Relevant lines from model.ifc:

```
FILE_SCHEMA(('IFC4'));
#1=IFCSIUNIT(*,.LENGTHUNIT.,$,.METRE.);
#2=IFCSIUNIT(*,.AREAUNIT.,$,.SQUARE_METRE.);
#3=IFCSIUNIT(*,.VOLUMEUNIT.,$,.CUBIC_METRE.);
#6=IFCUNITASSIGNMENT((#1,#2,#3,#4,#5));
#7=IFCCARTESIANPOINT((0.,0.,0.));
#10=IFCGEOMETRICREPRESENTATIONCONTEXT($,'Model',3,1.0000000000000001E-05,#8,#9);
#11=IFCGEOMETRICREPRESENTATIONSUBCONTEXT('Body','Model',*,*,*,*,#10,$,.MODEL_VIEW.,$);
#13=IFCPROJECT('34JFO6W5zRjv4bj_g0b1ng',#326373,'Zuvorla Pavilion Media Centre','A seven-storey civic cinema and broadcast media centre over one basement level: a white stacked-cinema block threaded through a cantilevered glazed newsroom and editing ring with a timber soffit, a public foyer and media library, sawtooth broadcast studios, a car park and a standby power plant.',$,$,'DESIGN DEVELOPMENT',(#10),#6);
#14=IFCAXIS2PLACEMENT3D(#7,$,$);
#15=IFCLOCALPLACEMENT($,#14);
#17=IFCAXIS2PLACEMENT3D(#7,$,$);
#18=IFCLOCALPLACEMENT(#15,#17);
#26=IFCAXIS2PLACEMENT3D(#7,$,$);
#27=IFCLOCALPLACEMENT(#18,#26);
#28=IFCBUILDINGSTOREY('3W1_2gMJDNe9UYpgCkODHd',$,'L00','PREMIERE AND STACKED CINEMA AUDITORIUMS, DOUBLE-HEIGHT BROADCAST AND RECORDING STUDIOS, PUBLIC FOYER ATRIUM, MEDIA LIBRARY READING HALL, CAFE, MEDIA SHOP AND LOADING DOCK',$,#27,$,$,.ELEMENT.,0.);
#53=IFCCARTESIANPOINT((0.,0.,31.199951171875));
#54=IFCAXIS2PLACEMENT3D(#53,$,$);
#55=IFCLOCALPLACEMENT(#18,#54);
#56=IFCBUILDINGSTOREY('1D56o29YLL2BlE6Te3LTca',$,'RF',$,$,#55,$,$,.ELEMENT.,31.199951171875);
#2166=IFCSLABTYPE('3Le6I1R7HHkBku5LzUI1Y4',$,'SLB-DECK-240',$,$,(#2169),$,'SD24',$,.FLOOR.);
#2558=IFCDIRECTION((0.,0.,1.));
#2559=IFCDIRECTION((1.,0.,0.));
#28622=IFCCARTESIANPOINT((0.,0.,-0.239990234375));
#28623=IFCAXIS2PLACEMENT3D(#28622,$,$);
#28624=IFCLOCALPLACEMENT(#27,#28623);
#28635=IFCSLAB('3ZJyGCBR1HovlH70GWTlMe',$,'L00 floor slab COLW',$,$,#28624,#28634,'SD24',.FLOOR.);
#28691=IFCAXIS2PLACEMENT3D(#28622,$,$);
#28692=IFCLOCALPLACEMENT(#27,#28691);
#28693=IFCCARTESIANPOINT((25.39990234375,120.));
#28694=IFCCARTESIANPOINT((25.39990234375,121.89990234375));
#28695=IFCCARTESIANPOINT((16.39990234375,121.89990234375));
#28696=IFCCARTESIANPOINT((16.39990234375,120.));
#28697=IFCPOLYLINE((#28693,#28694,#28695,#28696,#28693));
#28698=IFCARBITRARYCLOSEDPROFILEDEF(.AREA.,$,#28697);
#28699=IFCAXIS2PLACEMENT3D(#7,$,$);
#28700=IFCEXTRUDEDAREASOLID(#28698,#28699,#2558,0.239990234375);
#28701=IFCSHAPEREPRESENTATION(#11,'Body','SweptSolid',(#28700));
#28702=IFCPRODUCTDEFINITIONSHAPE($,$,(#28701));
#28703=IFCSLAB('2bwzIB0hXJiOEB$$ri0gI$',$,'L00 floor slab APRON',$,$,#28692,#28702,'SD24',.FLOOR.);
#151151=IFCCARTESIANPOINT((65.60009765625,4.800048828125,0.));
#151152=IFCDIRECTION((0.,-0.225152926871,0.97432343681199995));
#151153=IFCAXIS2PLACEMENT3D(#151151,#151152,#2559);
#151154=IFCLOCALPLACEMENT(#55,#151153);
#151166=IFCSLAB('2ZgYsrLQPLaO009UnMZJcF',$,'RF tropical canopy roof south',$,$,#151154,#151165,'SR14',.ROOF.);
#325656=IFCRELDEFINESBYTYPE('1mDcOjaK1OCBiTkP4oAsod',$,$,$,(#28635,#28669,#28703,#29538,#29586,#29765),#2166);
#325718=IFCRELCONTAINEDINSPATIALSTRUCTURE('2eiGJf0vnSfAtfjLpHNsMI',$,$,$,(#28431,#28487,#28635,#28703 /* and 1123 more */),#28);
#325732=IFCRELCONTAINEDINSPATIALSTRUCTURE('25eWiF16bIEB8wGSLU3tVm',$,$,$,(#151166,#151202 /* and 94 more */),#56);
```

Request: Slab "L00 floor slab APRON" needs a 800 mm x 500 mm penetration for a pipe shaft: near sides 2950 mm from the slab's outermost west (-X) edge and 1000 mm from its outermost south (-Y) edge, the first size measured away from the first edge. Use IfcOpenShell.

```python
import numpy as np
import ifcopenshell
import ifcopenshell.api.feature
import ifcopenshell.api.geometry
import ifcopenshell.api.root
import ifcopenshell.geom
import ifcopenshell.util.placement
import ifcopenshell.util.representation
import ifcopenshell.util.shape
import ifcopenshell.util.unit

model = ifcopenshell.open("model.ifc")
unit_scale = ifcopenshell.util.unit.calculate_unit_scale(model)
settings = ifcopenshell.geom.settings()


def volume(element):
    """Net volume in cubic metres, openings subtracted."""
    shape = ifcopenshell.geom.create_shape(settings, element)
    return ifcopenshell.util.shape.get_volume(shape.geometry)


slab = model.by_guid("2bwzIB0hXJiOEB$$ri0gI$")
before = volume(slab)

# Extent in the slab's own axes, in metres. The edges named are its -X and -Y sides.
slab_shape = ifcopenshell.geom.create_shape(settings, slab)
vertices = ifcopenshell.util.shape.get_vertices(slab_shape.geometry)
x_min, y_min, bottom = vertices.min(axis=0)
top = vertices[:, 2].max()

opening = ifcopenshell.api.root.create_entity(model, ifc_class="IfcOpeningElement", name="Pipe shaft opening", predefined_type="OPENING")
context = ifcopenshell.util.representation.get_context(model, "Model", "Body", "MODEL_VIEW")
width, depth = 0.8, 0.5
outline = [(0.0, 0.0), (width, 0.0), (width, depth), (0.0, depth), (0.0, 0.0)]
# Overshoot both faces by 50 mm so the cut is clean.
shape = ifcopenshell.api.geometry.add_slab_representation(
    model, context=context, depth=top - bottom + 0.1, polyline=outline
)
ifcopenshell.api.geometry.assign_representation(model, product=opening, representation=shape)

matrix = ifcopenshell.util.placement.get_local_placement(slab.ObjectPlacement)
matrix[:, 3] = matrix @ np.append(np.array([x_min + 2.95, y_min + 1, bottom - 0.05]) / unit_scale, 1.0)
ifcopenshell.api.geometry.edit_object_placement(model, product=opening, matrix=matrix, is_si=False)
ifcopenshell.api.feature.add_feature(model, feature=opening, element=slab)

after = volume(slab)

print(f"slab volume {before:.3f} -> {after:.3f} m3")

model.write("model_updated.ifc")
```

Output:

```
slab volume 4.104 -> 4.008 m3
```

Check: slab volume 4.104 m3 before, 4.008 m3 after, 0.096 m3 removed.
